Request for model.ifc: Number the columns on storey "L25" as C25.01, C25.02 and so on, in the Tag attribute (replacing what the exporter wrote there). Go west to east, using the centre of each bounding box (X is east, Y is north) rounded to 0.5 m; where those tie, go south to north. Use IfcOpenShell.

First a look at what the model holds.

```python
import ifcopenshell
import ifcopenshell.util.element
import ifcopenshell.util.placement

model = ifcopenshell.open("model.ifc")
print(model.schema)
storey = next(s for s in model.by_type("IfcBuildingStorey") if s.Name == "L25")
columns = [e for e in ifcopenshell.util.element.get_decomposition(storey) if e.is_a("IfcColumn")]
for e in sorted(columns, key=lambda e: e.id()):
    origin = ifcopenshell.util.placement.get_local_placement(e.ObjectPlacement)[:3, 3]
    print(e.id(), e.Tag, e.Name, origin.round(2) + 0.0, sep=" | ")
```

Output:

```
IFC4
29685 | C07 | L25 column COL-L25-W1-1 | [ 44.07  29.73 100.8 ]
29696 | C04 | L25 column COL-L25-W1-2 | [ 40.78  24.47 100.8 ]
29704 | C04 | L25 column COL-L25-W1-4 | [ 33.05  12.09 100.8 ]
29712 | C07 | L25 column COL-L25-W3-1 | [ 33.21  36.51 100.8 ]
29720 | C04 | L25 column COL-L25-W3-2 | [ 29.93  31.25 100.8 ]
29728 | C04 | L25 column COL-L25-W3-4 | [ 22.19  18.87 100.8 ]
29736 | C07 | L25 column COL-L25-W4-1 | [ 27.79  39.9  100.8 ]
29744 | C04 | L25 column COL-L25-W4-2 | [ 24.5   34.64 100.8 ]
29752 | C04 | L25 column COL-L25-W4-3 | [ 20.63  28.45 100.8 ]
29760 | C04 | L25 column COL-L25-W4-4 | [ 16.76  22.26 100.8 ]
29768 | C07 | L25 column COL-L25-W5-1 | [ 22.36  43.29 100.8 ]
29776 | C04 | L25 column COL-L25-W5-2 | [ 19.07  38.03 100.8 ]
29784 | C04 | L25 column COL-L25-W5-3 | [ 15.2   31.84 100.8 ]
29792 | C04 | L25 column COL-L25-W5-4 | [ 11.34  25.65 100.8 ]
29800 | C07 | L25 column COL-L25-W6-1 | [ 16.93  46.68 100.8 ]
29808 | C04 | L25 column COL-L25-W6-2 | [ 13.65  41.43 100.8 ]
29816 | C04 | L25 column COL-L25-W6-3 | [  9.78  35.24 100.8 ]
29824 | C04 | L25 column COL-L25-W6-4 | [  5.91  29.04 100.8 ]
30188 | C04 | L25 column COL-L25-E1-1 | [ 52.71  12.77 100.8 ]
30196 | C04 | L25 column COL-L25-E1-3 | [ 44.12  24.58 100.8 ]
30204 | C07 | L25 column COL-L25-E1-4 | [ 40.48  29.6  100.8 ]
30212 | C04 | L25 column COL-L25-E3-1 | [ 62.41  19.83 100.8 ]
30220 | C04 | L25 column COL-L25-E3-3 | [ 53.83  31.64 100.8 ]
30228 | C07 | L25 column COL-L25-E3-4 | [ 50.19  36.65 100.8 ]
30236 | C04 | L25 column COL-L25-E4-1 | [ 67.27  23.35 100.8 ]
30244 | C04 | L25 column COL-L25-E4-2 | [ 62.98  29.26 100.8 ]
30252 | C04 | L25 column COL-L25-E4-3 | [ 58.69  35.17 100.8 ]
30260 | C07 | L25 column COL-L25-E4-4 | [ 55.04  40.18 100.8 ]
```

```python
import ifcopenshell
import ifcopenshell.geom
import ifcopenshell.util.element
import ifcopenshell.util.shape

model = ifcopenshell.open("model.ifc")
settings = ifcopenshell.geom.settings()
settings.set("use-world-coords", True)


def centre(element):
    shape = ifcopenshell.geom.create_shape(settings, element)
    return ifcopenshell.util.shape.get_bbox_centroid(shape.geometry)


storey = next(s for s in model.by_type("IfcBuildingStorey") if s.Name == "L25")
columns = [e for e in ifcopenshell.util.element.get_decomposition(storey) if e.is_a("IfcColumn")]

# Insertion points can sit at a corner or the storey origin, so sort by the geometry (in metres).
centres = {e: centre(e) for e in columns}
columns.sort(key=lambda e: (round(centres[e][0] / 0.5), centres[e][1]))

for i, e in enumerate(columns, start=1):
    number = f"C25.{i:02d}"
    e.Tag = number
    print(e.id(), number)

model.write("model_edited.ifc")
```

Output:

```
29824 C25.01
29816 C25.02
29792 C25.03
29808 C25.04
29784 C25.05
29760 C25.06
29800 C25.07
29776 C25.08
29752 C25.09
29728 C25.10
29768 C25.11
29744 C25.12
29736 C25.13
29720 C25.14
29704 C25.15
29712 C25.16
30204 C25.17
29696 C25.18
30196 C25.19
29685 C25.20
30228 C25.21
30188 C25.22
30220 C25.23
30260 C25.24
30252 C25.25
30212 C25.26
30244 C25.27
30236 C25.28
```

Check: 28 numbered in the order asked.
